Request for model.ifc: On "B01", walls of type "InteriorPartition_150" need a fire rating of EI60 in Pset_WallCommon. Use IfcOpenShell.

First a look at what the model holds.

```python
import ifcopenshell
import ifcopenshell.util.element

model = ifcopenshell.open("model.ifc")
print(model.schema)
storey = next(s for s in model.by_type("IfcBuildingStorey") if s.Name == "B01")
walls = [e for e in ifcopenshell.util.element.get_decomposition(storey) if e.is_a("IfcWall")]
seen = {}
for e in walls:
    element_type = ifcopenshell.util.element.get_type(e)
    key = (element_type.Name if element_type != e and element_type else None, ifcopenshell.util.element.get_pset(e, "Pset_WallCommon", "FireRating"))
    seen[key] = seen.get(key, 0) + 1
for (name, value), count in sorted(seen.items(), key=str):
    print(count, "x", name, "|", value)
```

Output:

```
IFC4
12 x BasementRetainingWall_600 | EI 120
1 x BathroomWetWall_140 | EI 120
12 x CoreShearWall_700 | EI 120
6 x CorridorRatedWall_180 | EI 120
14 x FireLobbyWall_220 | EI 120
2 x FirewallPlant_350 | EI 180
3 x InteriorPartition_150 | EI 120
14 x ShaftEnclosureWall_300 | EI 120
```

```python
import ifcopenshell
import ifcopenshell.api.pset
import ifcopenshell.util.element

model = ifcopenshell.open("model.ifc")

storey = next(s for s in model.by_type("IfcBuildingStorey") if s.Name == "B01")
walls = [e for e in ifcopenshell.util.element.get_decomposition(storey) if e.is_a("IfcWall")]

count = 0
for e in walls:
    element_type = ifcopenshell.util.element.get_type(e)
    if element_type in (None, e) or element_type.Name != "InteriorPartition_150":
        continue
    # add_pset returns the element's existing set when there is one.
    pset = ifcopenshell.api.pset.add_pset(model, product=e, name="Pset_WallCommon")
    ifcopenshell.api.pset.edit_pset(model, pset=pset, properties={"FireRating": "EI60"})
    count += 1

print(count, "walls updated")

model.write("model-out.ifc")
```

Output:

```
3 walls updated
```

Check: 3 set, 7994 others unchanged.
